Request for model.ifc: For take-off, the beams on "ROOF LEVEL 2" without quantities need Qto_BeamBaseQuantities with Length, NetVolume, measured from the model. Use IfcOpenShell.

First a look at what the model holds.

```python
import ifcopenshell
import ifcopenshell.util.element
import ifcopenshell.util.unit

model = ifcopenshell.open("model.ifc")
print(model.schema)
for unit_type in ("LENGTHUNIT", "AREAUNIT", "VOLUMEUNIT"):
    print(unit_type, ifcopenshell.util.unit.calculate_unit_scale(model, unit_type))
storey = next(s for s in model.by_type("IfcBuildingStorey") if s.Name == "ROOF LEVEL 2")
beams = [e for e in ifcopenshell.util.element.get_decomposition(storey) if e.is_a("IfcBeam")]
for e in sorted(beams, key=lambda e: e.id()):
    print(e.id(), e.is_a(), e.Name, list(ifcopenshell.util.element.get_psets(e, qtos_only=True)), sep=" | ")
```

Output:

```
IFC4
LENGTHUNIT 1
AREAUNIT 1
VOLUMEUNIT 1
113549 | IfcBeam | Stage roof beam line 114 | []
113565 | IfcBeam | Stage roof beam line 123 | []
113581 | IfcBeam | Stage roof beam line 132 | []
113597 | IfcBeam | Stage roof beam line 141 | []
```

```python
import ifcopenshell
import ifcopenshell.api.pset
import ifcopenshell.geom
import ifcopenshell.util.element
import ifcopenshell.util.shape
import ifcopenshell.util.unit

model = ifcopenshell.open("model.ifc")
unit_scale = ifcopenshell.util.unit.calculate_unit_scale(model)
volume_scale = ifcopenshell.util.unit.calculate_unit_scale(model, "VOLUMEUNIT")
settings = ifcopenshell.geom.settings()

storey = next(s for s in model.by_type("IfcBuildingStorey") if s.Name == "ROOF LEVEL 2")
beams = [e for e in ifcopenshell.util.element.get_decomposition(storey) if e.is_a("IfcBeam")]

for e in sorted(beams, key=lambda e: e.id()):
    if ifcopenshell.util.element.get_psets(e, qtos_only=True, should_inherit=False):
        continue
    # Geometry comes back in metres, in the element's own axes.
    shape = ifcopenshell.geom.create_shape(settings, e)
    values = {
        "Length": ifcopenshell.util.shape.get_max_xyz(shape.geometry) / unit_scale,
        "NetVolume": ifcopenshell.util.shape.get_volume(shape.geometry) / volume_scale,
    }
    qto = ifcopenshell.api.pset.add_qto(model, product=e, name="Qto_BeamBaseQuantities")
    ifcopenshell.api.pset.edit_qto(model, qto=qto, properties=values)
    print(e.id(), {k: round(v, 3) for k, v in values.items()})

model.write("model_edited.ifc")
```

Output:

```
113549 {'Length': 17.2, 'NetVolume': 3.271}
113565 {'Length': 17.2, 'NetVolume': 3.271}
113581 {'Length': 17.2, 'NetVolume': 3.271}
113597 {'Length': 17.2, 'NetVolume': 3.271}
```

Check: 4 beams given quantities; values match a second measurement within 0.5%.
